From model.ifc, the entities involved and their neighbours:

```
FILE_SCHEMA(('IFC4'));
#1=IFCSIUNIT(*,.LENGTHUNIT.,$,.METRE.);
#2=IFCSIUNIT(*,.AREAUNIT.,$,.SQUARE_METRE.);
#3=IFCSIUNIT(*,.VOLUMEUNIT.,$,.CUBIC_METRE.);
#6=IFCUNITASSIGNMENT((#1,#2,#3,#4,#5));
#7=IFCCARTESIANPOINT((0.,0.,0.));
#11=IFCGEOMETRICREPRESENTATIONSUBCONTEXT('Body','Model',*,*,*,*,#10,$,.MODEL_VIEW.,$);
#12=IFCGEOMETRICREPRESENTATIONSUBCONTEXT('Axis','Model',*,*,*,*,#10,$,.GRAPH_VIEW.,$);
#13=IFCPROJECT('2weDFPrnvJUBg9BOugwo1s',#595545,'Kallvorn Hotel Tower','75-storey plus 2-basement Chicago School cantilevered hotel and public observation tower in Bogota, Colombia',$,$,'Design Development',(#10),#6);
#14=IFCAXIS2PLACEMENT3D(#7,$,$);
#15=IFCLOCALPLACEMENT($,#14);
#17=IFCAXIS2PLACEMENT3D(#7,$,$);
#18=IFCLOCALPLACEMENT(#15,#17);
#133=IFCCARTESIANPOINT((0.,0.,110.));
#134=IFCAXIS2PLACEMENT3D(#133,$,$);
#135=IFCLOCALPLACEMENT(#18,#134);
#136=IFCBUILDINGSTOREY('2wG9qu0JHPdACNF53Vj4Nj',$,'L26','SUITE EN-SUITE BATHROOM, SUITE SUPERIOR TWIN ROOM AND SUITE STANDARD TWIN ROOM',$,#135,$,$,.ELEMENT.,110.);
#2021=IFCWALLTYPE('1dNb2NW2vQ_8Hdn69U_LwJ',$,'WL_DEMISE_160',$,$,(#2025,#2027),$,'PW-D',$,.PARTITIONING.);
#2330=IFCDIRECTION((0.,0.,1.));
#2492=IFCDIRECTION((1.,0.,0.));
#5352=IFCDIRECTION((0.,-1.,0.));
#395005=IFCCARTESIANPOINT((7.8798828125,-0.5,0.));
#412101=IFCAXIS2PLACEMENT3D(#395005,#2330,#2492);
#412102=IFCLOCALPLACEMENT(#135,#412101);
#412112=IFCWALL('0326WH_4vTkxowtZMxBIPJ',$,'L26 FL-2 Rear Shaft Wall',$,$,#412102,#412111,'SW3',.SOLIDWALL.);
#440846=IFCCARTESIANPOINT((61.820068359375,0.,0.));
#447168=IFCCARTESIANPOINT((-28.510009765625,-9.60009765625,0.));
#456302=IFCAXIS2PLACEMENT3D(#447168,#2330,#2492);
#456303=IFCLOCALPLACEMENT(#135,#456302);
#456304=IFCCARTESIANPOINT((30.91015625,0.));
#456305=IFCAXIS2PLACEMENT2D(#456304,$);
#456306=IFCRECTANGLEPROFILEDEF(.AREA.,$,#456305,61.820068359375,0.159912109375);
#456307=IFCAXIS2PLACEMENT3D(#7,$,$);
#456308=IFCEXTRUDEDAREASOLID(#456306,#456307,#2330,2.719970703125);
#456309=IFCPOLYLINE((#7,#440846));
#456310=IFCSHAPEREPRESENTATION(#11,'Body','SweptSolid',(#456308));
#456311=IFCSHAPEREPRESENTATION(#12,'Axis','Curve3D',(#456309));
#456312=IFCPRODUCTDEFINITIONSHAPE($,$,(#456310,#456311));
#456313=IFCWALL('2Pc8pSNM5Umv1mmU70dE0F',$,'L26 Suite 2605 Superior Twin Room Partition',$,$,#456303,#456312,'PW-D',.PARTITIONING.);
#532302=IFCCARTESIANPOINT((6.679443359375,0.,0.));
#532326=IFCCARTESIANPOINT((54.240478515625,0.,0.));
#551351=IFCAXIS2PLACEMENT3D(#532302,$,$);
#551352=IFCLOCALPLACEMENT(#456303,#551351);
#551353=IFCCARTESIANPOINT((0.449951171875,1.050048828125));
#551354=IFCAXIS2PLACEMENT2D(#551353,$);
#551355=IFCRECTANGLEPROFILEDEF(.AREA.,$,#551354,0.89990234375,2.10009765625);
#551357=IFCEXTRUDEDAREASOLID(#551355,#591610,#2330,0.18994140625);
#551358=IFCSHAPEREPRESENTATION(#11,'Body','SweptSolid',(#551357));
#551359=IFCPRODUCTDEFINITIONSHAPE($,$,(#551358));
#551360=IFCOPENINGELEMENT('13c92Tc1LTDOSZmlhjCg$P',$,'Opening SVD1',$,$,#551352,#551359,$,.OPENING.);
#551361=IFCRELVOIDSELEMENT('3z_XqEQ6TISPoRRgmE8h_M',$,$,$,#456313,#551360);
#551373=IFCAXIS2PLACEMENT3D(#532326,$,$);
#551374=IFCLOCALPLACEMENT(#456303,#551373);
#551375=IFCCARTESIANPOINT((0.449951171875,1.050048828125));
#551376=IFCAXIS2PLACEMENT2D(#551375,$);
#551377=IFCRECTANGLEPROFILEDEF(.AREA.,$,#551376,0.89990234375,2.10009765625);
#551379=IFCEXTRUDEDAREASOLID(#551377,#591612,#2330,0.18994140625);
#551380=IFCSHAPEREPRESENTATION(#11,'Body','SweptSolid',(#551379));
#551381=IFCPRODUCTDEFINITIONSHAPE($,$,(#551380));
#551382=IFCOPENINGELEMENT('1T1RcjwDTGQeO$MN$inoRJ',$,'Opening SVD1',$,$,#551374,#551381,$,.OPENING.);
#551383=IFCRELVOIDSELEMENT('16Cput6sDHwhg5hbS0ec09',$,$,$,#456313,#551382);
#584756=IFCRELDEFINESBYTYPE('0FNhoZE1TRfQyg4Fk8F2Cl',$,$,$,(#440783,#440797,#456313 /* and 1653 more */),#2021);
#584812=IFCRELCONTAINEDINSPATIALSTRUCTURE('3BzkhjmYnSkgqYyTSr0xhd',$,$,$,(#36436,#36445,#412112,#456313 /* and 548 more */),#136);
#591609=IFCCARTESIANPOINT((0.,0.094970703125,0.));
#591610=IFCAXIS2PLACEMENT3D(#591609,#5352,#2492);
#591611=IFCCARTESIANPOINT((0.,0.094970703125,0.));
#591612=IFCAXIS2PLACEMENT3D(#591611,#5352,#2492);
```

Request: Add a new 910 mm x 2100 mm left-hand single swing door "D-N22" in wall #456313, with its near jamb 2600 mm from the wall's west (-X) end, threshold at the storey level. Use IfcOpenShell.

```python
import numpy as np
import ifcopenshell
import ifcopenshell.api.feature
import ifcopenshell.api.geometry
import ifcopenshell.api.root
import ifcopenshell.api.spatial
import ifcopenshell.geom
import ifcopenshell.util.element
import ifcopenshell.util.placement
import ifcopenshell.util.representation
import ifcopenshell.util.shape
import ifcopenshell.util.unit

model = ifcopenshell.open("model.ifc")
unit_scale = ifcopenshell.util.unit.calculate_unit_scale(model)
settings = ifcopenshell.geom.settings()


def volume(element):
    """Net volume in cubic metres, openings subtracted."""
    shape = ifcopenshell.geom.create_shape(settings, element)
    return ifcopenshell.util.shape.get_volume(shape.geometry)


wall = model.by_guid("2Pc8pSNM5Umv1mmU70dE0F")
storey = ifcopenshell.util.element.get_container(wall, ifc_class="IfcBuildingStorey")
context = ifcopenshell.util.representation.get_context(model, "Model", "Body", "MODEL_VIEW")
before = volume(wall)

width, height, from_end, sill = 0.91, 2.1, 2.6, 0.0  # metres

# The wall runs along its own X axis, and the end named is its -X end.
wall_shape = ifcopenshell.geom.create_shape(settings, wall)
x, y, z = ifcopenshell.util.shape.get_vertices(wall_shape.geometry).T
start = x.min() + from_end
face, thickness = float(y.min()), float(y.max() - y.min())
wall_matrix = ifcopenshell.util.placement.get_local_placement(wall.ObjectPlacement)
level = ifcopenshell.util.placement.get_local_placement(storey.ObjectPlacement)[2, 3]


def in_wall(x, y):
    """Placement at x, y metres in the wall's axes, at sill height."""
    matrix = wall_matrix.copy()
    matrix[:, 3] = wall_matrix @ np.array([x / unit_scale, y / unit_scale, 0.0, 1.0])
    matrix[2, 3] = level + sill / unit_scale
    return matrix


# Opening: a box that overshoots both wall faces by 50 mm.
opening = ifcopenshell.api.root.create_entity(model, ifc_class="IfcOpeningElement", predefined_type="OPENING")
box = ifcopenshell.api.geometry.add_wall_representation(
    model, context=context, length=width, height=height, thickness=thickness + 0.1
)
ifcopenshell.api.geometry.assign_representation(model, product=opening, representation=box)
ifcopenshell.api.geometry.edit_object_placement(model, product=opening, matrix=in_wall(start, face - 0.05), is_si=False)
ifcopenshell.api.feature.add_feature(model, feature=opening, element=wall)

door = ifcopenshell.api.root.create_entity(model, ifc_class="IfcDoor", name="D-N22", predefined_type="DOOR")
door.OverallWidth, door.OverallHeight = width / unit_scale, height / unit_scale
door.OperationType = "SINGLE_SWING_LEFT"
body = ifcopenshell.api.geometry.add_door_representation(
    model,
    context=context,
    overall_width=door.OverallWidth,
    overall_height=door.OverallHeight,
    operation_type="SINGLE_SWING_LEFT",
    lining_properties={"LiningDepth": thickness / unit_scale, "ThresholdDepth": thickness / unit_scale},
)
ifcopenshell.api.geometry.assign_representation(model, product=door, representation=body)
ifcopenshell.api.spatial.assign_container(model, products=[door], relating_structure=storey)
ifcopenshell.api.feature.add_filling(model, opening=opening, element=door)

# The lining spans the wall, so the door starts at the wall face.
ifcopenshell.api.geometry.edit_object_placement(model, product=door, matrix=in_wall(start, face), is_si=False)

after = volume(wall)

print(f"wall volume {before:.3f} -> {after:.3f} m3")

model.write("model-out.ifc")
```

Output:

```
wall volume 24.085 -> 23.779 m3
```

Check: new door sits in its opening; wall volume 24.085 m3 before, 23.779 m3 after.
